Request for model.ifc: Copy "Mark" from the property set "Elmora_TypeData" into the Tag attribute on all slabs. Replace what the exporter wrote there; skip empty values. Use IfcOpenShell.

First a look at what the model holds.

```python
import ifcopenshell
import ifcopenshell.util.element

model = ifcopenshell.open("model.ifc")
print(model.schema)
slabs = model.by_type("IfcSlab")
print(len(slabs), "slabs")
for e in slabs[:8]:
    source = ifcopenshell.util.element.get_pset(e, "Elmora_TypeData", "Mark")
    target = e.Tag
    print(e.id(), repr(source), repr(target), sep=" | ")
```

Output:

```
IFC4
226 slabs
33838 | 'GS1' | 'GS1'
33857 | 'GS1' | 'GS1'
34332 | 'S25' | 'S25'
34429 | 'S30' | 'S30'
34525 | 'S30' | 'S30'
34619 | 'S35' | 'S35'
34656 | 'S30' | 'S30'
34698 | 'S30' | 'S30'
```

```python
import ifcopenshell
import ifcopenshell.util.element

model = ifcopenshell.open("model.ifc")

count = 0
for e in model.by_type("IfcSlab"):
    value = ifcopenshell.util.element.get_pset(e, "Elmora_TypeData", "Mark")
    current = e.Tag
    if not value or not value.strip() or current == value:
        continue
    e.Tag = value
    count += 1

print(count, "slabs updated")

model.write("model_v2.ifc")
```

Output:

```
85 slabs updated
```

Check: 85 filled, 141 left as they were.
